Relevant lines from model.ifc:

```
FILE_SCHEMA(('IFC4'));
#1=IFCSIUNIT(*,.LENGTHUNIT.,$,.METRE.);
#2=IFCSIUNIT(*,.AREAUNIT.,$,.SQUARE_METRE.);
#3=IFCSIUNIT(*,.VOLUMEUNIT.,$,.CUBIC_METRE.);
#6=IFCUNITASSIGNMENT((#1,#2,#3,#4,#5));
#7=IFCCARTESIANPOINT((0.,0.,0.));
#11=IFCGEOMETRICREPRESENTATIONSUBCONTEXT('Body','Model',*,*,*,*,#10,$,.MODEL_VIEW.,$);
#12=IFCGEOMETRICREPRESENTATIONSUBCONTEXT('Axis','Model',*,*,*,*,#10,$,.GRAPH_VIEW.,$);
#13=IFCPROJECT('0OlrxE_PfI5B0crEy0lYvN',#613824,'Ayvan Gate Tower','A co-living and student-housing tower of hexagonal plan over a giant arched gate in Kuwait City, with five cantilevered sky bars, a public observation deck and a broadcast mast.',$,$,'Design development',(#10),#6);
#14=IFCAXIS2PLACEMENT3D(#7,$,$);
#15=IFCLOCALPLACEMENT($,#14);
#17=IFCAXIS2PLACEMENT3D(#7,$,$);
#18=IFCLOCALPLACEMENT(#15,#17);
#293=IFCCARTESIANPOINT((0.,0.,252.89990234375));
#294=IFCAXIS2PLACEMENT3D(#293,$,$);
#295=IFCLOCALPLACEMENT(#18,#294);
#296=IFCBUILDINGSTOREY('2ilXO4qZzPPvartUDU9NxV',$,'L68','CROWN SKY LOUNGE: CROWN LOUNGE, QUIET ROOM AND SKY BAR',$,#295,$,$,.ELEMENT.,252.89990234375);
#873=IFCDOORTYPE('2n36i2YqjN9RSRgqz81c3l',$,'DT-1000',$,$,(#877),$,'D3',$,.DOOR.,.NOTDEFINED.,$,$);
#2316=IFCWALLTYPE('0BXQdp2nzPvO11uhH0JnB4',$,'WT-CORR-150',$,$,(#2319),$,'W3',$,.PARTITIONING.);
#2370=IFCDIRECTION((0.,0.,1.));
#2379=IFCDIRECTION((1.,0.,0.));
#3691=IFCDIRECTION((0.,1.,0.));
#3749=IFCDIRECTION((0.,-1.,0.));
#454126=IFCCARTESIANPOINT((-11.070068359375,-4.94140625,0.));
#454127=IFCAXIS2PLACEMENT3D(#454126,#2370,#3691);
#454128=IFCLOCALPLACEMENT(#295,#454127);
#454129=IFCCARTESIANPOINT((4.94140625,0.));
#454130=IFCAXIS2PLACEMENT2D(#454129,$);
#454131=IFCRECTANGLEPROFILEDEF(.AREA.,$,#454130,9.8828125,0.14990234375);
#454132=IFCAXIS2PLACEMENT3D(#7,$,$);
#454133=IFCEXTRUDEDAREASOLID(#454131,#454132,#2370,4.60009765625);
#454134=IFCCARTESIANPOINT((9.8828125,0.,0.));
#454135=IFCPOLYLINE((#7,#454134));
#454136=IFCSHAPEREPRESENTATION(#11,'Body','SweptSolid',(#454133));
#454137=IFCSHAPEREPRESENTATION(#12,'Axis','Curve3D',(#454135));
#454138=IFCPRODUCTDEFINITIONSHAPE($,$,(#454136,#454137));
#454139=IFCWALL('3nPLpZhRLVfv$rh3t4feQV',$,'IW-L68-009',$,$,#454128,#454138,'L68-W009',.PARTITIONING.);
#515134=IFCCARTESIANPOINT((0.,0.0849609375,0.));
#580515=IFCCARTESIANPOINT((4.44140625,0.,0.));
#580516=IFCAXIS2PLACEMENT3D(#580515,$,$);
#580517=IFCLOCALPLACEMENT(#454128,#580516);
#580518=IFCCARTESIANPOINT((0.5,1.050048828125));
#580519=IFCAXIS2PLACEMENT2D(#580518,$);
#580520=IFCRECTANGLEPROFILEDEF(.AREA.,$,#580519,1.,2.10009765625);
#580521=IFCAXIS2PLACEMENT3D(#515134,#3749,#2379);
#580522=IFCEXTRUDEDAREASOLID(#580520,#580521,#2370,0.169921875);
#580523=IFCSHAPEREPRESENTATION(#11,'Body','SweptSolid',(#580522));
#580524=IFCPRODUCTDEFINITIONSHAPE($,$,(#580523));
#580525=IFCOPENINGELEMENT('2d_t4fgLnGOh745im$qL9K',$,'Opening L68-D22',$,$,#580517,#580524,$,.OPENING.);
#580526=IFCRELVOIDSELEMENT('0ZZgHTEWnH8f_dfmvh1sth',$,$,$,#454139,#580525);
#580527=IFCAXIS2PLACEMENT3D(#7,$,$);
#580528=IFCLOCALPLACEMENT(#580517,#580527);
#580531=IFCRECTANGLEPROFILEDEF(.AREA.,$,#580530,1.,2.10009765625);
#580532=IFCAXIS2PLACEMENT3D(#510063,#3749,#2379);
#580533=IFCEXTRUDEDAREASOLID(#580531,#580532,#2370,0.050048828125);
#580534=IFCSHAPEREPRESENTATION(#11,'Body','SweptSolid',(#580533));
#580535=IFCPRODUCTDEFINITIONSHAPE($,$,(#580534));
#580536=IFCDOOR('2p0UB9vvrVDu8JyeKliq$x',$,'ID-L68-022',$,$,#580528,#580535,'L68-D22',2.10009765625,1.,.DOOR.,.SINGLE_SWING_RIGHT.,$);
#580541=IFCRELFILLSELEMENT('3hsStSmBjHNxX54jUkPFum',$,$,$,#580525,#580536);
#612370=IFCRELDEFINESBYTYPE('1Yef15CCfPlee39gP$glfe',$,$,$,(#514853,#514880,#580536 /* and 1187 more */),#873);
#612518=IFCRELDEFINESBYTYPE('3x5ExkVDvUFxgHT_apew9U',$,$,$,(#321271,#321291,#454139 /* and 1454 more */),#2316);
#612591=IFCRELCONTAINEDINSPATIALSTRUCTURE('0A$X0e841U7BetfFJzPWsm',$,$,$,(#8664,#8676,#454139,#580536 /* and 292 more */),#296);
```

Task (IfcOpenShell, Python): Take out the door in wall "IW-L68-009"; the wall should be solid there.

```python
import ifcopenshell
import ifcopenshell.api.feature
import ifcopenshell.api.root
import ifcopenshell.geom
import ifcopenshell.util.shape

model = ifcopenshell.open("model.ifc")
settings = ifcopenshell.geom.settings()


def volume(element):
    """Net volume in cubic metres, openings subtracted."""
    shape = ifcopenshell.geom.create_shape(settings, element)
    return ifcopenshell.util.shape.get_volume(shape.geometry)


door = model.by_guid("2p0UB9vvrVDu8JyeKliq$x")
opening = door.FillsVoids[0].RelatingOpeningElement
wall = opening.VoidsElements[0].RelatingBuildingElement
before = volume(wall)

ifcopenshell.api.root.remove_product(model, product=door)
ifcopenshell.api.feature.remove_feature(model, feature=opening)

after = volume(wall)

print(f"wall volume {before:.3f} -> {after:.3f} m3")

model.write("model_rev.ifc")
```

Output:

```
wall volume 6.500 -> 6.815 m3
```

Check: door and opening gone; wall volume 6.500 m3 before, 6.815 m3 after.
